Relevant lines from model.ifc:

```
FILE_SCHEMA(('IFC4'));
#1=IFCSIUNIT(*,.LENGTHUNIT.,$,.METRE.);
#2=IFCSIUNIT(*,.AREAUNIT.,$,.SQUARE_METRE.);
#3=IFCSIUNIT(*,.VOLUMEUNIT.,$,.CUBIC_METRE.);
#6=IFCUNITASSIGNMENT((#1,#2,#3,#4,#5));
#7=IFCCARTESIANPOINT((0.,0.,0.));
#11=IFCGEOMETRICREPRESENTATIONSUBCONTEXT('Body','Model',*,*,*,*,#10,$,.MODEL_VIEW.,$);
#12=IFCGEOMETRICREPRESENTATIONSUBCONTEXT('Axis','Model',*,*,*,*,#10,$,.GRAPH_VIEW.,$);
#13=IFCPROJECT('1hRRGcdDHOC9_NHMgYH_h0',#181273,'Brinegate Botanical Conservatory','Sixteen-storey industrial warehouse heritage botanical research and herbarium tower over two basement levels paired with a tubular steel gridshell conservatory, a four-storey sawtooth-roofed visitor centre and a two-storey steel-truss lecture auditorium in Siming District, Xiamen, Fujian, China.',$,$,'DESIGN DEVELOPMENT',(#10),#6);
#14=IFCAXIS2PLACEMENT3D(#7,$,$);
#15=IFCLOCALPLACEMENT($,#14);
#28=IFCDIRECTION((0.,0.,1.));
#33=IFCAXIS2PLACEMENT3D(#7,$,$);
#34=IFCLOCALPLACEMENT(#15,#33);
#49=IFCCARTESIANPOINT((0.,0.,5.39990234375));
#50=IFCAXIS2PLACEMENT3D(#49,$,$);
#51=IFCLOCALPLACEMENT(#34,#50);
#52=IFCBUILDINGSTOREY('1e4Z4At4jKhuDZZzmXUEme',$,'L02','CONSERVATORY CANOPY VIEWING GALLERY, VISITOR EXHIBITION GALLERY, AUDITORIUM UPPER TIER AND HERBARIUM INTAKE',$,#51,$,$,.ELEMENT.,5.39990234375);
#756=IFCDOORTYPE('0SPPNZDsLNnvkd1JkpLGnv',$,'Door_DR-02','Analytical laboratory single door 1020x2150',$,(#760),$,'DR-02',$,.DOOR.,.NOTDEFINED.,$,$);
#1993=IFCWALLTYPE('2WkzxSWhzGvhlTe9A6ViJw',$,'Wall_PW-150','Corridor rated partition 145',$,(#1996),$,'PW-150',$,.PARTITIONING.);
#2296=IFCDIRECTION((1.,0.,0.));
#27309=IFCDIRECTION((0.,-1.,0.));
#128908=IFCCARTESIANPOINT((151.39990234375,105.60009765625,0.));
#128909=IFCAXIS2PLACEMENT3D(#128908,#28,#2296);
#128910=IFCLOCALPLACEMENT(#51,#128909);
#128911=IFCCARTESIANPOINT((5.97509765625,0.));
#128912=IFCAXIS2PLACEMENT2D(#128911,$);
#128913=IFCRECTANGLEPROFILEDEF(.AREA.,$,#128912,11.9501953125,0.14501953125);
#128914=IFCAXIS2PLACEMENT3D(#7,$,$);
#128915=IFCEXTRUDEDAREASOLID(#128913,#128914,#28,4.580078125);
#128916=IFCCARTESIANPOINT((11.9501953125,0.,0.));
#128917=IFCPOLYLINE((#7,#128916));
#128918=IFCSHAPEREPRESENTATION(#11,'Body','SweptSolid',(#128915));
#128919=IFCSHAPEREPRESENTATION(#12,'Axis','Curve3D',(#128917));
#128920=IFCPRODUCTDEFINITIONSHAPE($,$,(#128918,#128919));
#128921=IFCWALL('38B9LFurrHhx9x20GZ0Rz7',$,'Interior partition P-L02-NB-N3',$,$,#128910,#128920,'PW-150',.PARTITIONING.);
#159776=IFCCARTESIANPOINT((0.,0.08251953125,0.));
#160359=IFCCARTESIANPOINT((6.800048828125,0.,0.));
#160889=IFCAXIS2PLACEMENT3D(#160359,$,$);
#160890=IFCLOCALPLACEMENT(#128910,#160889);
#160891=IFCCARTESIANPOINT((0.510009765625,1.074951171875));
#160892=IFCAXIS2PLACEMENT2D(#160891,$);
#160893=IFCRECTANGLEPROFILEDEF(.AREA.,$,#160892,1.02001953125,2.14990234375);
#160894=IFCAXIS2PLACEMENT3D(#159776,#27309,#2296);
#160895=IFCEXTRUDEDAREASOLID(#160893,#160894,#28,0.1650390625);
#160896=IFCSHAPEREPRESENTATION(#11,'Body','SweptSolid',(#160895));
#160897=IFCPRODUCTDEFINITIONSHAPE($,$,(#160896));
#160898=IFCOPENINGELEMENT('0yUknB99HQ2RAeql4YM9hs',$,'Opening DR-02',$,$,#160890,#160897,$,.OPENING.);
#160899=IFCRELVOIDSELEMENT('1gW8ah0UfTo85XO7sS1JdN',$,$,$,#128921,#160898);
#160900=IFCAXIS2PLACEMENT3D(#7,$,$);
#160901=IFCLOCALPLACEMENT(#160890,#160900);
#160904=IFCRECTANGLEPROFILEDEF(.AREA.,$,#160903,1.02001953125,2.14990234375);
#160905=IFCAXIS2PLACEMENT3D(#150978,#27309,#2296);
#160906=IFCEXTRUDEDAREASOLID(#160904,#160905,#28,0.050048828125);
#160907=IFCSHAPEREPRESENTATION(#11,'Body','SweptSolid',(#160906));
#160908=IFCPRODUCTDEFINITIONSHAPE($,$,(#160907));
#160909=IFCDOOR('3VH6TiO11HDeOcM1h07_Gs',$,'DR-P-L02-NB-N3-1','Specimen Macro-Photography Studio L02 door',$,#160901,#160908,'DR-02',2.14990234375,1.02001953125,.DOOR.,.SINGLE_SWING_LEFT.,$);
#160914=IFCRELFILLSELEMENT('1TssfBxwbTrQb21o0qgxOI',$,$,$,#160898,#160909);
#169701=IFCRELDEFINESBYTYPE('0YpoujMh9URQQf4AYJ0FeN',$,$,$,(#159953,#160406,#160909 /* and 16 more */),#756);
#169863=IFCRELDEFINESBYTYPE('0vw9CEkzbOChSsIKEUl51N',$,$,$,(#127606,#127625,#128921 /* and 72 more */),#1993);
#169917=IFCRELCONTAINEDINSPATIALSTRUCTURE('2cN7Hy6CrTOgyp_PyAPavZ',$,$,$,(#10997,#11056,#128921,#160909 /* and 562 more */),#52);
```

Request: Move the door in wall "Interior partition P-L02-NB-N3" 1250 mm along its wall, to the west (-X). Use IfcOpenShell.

```python
import ifcopenshell
import ifcopenshell.api.geometry
import ifcopenshell.util.placement
import ifcopenshell.util.unit

model = ifcopenshell.open("model.ifc")
unit_scale = ifcopenshell.util.unit.calculate_unit_scale(model)

door = model.by_id(160909)
opening = door.FillsVoids[0].RelatingOpeningElement
wall = opening.VoidsElements[0].RelatingBuildingElement

wall_matrix = ifcopenshell.util.placement.get_local_placement(wall.ObjectPlacement)
shift = wall_matrix[:3, 0] * -1.25 / unit_scale
before = ifcopenshell.util.placement.get_local_placement(door.ObjectPlacement)[:3, 3].copy()

# The door is placed relative to its opening, so it follows when the opening moves.
matrix = ifcopenshell.util.placement.get_local_placement(opening.ObjectPlacement)
matrix[:3, 3] += shift
ifcopenshell.api.geometry.edit_object_placement(
    model, product=opening, matrix=matrix, is_si=False, should_transform_children=True
)

after = ifcopenshell.util.placement.get_local_placement(door.ObjectPlacement)[:3, 3]
print("door moved by", (after - before).round(3) + 0.0)

model.write("model_edited.ifc")
```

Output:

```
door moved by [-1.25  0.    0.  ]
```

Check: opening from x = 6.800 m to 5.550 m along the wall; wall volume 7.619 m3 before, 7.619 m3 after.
